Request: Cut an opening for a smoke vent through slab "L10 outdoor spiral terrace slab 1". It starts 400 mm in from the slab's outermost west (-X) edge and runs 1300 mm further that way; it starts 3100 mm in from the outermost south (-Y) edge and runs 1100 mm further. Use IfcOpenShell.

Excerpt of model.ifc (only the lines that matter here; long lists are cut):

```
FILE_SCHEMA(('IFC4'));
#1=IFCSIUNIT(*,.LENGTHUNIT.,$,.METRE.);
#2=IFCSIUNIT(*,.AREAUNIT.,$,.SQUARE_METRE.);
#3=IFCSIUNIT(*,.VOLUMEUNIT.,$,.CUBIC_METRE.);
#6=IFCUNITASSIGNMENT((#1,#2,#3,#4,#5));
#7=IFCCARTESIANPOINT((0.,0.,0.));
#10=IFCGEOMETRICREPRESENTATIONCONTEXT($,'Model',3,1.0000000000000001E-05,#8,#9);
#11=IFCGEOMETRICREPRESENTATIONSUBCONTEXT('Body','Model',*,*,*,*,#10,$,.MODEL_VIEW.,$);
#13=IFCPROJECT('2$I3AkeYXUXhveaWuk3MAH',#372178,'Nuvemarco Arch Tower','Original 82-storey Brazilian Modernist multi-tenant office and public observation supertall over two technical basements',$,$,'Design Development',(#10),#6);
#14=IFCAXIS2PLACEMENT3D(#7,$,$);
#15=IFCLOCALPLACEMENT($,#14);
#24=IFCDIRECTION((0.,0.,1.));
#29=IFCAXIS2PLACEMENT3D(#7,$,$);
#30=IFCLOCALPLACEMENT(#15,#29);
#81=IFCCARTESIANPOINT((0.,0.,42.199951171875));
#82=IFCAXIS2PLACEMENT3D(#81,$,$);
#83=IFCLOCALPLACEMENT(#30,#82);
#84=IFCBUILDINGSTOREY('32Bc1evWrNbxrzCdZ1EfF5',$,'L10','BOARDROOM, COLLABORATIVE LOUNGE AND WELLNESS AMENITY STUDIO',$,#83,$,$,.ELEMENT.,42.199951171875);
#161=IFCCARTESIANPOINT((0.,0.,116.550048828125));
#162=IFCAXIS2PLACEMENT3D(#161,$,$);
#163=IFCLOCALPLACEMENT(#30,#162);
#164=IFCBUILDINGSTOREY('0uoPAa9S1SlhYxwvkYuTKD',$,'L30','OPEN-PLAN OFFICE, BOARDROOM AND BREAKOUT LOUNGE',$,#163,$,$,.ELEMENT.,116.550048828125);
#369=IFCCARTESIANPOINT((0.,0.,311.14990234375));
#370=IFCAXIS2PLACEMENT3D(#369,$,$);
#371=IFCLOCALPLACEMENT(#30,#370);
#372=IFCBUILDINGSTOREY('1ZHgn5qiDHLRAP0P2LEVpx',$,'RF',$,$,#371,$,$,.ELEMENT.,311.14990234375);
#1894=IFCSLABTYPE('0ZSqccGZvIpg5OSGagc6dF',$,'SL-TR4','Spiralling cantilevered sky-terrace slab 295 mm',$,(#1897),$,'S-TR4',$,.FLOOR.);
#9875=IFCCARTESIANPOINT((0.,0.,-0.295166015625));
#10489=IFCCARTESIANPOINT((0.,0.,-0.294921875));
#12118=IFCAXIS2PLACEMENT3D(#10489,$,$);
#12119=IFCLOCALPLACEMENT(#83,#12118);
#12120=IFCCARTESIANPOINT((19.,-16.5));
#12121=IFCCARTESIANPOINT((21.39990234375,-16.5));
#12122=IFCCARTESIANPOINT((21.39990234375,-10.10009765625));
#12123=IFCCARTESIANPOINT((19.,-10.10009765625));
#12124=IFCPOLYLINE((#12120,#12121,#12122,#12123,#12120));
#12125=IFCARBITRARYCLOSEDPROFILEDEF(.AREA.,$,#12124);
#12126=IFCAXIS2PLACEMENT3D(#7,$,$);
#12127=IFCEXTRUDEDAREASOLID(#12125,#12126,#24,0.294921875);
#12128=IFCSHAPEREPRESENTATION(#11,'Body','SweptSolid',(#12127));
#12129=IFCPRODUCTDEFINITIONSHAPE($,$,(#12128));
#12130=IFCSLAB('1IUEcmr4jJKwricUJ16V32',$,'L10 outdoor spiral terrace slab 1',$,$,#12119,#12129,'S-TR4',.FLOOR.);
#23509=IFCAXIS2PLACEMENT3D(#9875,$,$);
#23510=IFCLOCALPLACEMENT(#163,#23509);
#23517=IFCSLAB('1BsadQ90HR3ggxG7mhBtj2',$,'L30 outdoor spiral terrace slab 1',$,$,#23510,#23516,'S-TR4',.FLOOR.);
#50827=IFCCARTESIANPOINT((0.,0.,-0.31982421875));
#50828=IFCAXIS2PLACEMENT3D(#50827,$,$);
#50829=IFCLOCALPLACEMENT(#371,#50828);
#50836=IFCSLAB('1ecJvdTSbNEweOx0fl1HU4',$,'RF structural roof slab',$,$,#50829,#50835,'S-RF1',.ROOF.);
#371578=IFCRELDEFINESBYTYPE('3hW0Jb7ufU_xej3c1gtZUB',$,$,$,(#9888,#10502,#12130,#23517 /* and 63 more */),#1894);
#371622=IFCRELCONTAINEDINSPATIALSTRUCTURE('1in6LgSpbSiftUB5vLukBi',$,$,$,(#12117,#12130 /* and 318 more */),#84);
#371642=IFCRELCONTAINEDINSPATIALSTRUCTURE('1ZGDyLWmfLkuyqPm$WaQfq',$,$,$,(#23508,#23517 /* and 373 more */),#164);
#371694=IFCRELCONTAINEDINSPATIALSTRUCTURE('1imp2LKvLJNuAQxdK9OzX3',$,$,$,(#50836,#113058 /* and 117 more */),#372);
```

```python
import numpy as np
import ifcopenshell
import ifcopenshell.api.feature
import ifcopenshell.api.geometry
import ifcopenshell.api.root
import ifcopenshell.geom
import ifcopenshell.util.placement
import ifcopenshell.util.representation
import ifcopenshell.util.shape
import ifcopenshell.util.unit

model = ifcopenshell.open("model.ifc")
unit_scale = ifcopenshell.util.unit.calculate_unit_scale(model)
settings = ifcopenshell.geom.settings()


def volume(element):
    """Net volume in cubic metres, openings subtracted."""
    shape = ifcopenshell.geom.create_shape(settings, element)
    return ifcopenshell.util.shape.get_volume(shape.geometry)


slab = model.by_guid("1IUEcmr4jJKwricUJ16V32")
before = volume(slab)

# Extent in the slab's own axes, in metres. The edges named are its -X and -Y sides.
slab_shape = ifcopenshell.geom.create_shape(settings, slab)
vertices = ifcopenshell.util.shape.get_vertices(slab_shape.geometry)
x_min, y_min, bottom = vertices.min(axis=0)
top = vertices[:, 2].max()

opening = ifcopenshell.api.root.create_entity(model, ifc_class="IfcOpeningElement", name="Smoke vent opening", predefined_type="OPENING")
context = ifcopenshell.util.representation.get_context(model, "Model", "Body", "MODEL_VIEW")
width, depth = 1.3, 1.1
outline = [(0.0, 0.0), (width, 0.0), (width, depth), (0.0, depth), (0.0, 0.0)]
# Overshoot both faces by 50 mm so the cut is clean.
shape = ifcopenshell.api.geometry.add_slab_representation(
    model, context=context, depth=top - bottom + 0.1, polyline=outline
)
ifcopenshell.api.geometry.assign_representation(model, product=opening, representation=shape)

matrix = ifcopenshell.util.placement.get_local_placement(slab.ObjectPlacement)
matrix[:, 3] = matrix @ np.append(np.array([x_min + 0.4, y_min + 3.1, bottom - 0.05]) / unit_scale, 1.0)
ifcopenshell.api.geometry.edit_object_placement(model, product=opening, matrix=matrix, is_si=False)
ifcopenshell.api.feature.add_feature(model, feature=opening, element=slab)

after = volume(slab)

print(f"slab volume {before:.3f} -> {after:.3f} m3")

model.write("model-out.ifc")
```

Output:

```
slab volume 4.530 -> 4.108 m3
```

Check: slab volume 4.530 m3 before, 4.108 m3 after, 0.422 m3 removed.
